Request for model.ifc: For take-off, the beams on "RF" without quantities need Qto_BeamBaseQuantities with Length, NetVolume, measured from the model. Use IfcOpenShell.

First a look at what the model holds.

```python
import ifcopenshell
import ifcopenshell.util.element
import ifcopenshell.util.unit

model = ifcopenshell.open("model.ifc")
print(model.schema)
for unit_type in ("LENGTHUNIT", "AREAUNIT", "VOLUMEUNIT"):
    print(unit_type, ifcopenshell.util.unit.calculate_unit_scale(model, unit_type))
storey = next(s for s in model.by_type("IfcBuildingStorey") if s.Name == "RF")
beams = [e for e in ifcopenshell.util.element.get_decomposition(storey) if e.is_a("IfcBeam")]
for e in sorted(beams, key=lambda e: e.id()):
    print(e.id(), e.is_a(), e.Name, list(ifcopenshell.util.element.get_psets(e, qtos_only=True)), sep=" | ")
```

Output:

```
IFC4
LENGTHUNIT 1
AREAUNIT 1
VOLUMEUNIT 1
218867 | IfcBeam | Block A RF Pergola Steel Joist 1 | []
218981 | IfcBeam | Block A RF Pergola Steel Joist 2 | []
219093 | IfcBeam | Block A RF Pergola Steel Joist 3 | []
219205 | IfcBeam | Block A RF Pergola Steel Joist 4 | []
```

```python
import ifcopenshell
import ifcopenshell.api.pset
import ifcopenshell.geom
import ifcopenshell.util.element
import ifcopenshell.util.shape
import ifcopenshell.util.unit

model = ifcopenshell.open("model.ifc")
unit_scale = ifcopenshell.util.unit.calculate_unit_scale(model)
volume_scale = ifcopenshell.util.unit.calculate_unit_scale(model, "VOLUMEUNIT")
settings = ifcopenshell.geom.settings()

storey = next(s for s in model.by_type("IfcBuildingStorey") if s.Name == "RF")
beams = [e for e in ifcopenshell.util.element.get_decomposition(storey) if e.is_a("IfcBeam")]

for e in sorted(beams, key=lambda e: e.id()):
    if ifcopenshell.util.element.get_psets(e, qtos_only=True, should_inherit=False):
        continue
    # Geometry comes back in metres, in the element's own axes.
    shape = ifcopenshell.geom.create_shape(settings, e)
    values = {
        "Length": ifcopenshell.util.shape.get_max_xyz(shape.geometry) / unit_scale,
        "NetVolume": ifcopenshell.util.shape.get_volume(shape.geometry) / volume_scale,
    }
    qto = ifcopenshell.api.pset.add_qto(model, product=e, name="Qto_BeamBaseQuantities")
    ifcopenshell.api.pset.edit_qto(model, qto=qto, properties=values)
    print(e.id(), {k: round(v, 3) for k, v in values.items()})

model.write("model_v2.ifc")
```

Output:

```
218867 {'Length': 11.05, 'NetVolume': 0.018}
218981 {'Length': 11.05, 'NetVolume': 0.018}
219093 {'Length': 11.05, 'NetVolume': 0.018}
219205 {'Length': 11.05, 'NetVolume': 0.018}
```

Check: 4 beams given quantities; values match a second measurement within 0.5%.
